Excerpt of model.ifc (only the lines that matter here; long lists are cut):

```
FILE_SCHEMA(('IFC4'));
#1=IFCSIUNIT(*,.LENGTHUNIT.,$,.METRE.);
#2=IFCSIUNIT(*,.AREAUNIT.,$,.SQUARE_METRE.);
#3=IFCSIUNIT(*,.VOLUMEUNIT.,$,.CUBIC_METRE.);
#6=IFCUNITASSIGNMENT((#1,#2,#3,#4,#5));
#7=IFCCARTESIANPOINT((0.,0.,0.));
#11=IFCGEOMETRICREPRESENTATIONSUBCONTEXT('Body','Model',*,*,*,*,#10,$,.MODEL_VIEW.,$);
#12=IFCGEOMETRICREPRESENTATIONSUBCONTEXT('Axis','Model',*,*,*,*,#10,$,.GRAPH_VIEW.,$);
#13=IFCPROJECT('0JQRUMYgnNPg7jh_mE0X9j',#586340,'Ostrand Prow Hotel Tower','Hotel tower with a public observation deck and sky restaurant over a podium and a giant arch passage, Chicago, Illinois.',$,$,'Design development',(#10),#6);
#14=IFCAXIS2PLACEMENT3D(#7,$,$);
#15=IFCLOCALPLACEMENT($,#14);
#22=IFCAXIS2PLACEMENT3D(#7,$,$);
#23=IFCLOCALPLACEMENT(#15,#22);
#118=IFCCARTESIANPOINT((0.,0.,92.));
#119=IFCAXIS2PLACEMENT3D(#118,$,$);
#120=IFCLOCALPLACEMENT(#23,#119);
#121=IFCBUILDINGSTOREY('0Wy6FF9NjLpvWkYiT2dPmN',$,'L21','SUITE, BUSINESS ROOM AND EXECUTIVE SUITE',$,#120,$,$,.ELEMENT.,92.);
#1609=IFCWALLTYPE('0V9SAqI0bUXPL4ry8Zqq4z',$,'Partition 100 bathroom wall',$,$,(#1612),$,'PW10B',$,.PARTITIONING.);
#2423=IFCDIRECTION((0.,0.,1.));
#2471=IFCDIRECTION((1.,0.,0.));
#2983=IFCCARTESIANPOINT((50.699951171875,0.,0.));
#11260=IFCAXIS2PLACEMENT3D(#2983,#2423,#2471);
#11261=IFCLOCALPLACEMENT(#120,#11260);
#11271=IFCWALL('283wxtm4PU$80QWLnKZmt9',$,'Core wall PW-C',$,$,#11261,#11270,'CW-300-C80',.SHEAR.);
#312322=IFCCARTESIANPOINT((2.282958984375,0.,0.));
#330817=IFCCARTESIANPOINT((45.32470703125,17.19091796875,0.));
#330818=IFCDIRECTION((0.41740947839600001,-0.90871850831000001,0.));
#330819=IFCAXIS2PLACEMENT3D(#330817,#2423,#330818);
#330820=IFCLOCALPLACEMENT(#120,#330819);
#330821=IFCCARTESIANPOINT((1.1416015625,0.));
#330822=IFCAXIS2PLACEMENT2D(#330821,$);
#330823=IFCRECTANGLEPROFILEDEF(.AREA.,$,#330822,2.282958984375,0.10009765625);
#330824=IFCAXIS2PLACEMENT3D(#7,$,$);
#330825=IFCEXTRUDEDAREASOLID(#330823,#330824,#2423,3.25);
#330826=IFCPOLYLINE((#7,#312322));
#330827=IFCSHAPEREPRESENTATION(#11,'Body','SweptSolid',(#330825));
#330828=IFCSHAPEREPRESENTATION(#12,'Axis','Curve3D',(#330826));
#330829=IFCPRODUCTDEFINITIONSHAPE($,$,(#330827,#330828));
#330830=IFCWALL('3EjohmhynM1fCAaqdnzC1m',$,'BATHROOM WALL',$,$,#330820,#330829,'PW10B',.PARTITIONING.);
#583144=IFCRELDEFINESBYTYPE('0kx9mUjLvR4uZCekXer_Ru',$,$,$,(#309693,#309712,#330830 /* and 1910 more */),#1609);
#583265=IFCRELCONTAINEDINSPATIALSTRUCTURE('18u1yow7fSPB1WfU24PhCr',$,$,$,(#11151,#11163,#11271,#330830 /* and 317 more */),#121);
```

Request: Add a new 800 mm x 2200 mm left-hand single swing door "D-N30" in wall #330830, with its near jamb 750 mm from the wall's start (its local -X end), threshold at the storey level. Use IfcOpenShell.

```python
import numpy as np
import ifcopenshell
import ifcopenshell.api.feature
import ifcopenshell.api.geometry
import ifcopenshell.api.root
import ifcopenshell.api.spatial
import ifcopenshell.geom
import ifcopenshell.util.element
import ifcopenshell.util.placement
import ifcopenshell.util.representation
import ifcopenshell.util.shape
import ifcopenshell.util.unit

model = ifcopenshell.open("model.ifc")
unit_scale = ifcopenshell.util.unit.calculate_unit_scale(model)
settings = ifcopenshell.geom.settings()


def volume(element):
    """Net volume in cubic metres, openings subtracted."""
    shape = ifcopenshell.geom.create_shape(settings, element)
    return ifcopenshell.util.shape.get_volume(shape.geometry)


wall = model.by_guid("3EjohmhynM1fCAaqdnzC1m")
storey = ifcopenshell.util.element.get_container(wall, ifc_class="IfcBuildingStorey")
context = ifcopenshell.util.representation.get_context(model, "Model", "Body", "MODEL_VIEW")
before = volume(wall)

width, height, from_end, sill = 0.8, 2.2, 0.75, 0.0  # metres

# The wall runs along its own X axis, and the end named is its -X end.
wall_shape = ifcopenshell.geom.create_shape(settings, wall)
x, y, z = ifcopenshell.util.shape.get_vertices(wall_shape.geometry).T
start = x.min() + from_end
face, thickness = float(y.min()), float(y.max() - y.min())
wall_matrix = ifcopenshell.util.placement.get_local_placement(wall.ObjectPlacement)
level = ifcopenshell.util.placement.get_local_placement(storey.ObjectPlacement)[2, 3]


def in_wall(x, y):
    """Placement at x, y metres in the wall's axes, at sill height."""
    matrix = wall_matrix.copy()
    matrix[:, 3] = wall_matrix @ np.array([x / unit_scale, y / unit_scale, 0.0, 1.0])
    matrix[2, 3] = level + sill / unit_scale
    return matrix


# Opening: a box that overshoots both wall faces by 50 mm.
opening = ifcopenshell.api.root.create_entity(model, ifc_class="IfcOpeningElement", predefined_type="OPENING")
box = ifcopenshell.api.geometry.add_wall_representation(
    model, context=context, length=width, height=height, thickness=thickness + 0.1
)
ifcopenshell.api.geometry.assign_representation(model, product=opening, representation=box)
ifcopenshell.api.geometry.edit_object_placement(model, product=opening, matrix=in_wall(start, face - 0.05), is_si=False)
ifcopenshell.api.feature.add_feature(model, feature=opening, element=wall)

door = ifcopenshell.api.root.create_entity(model, ifc_class="IfcDoor", name="D-N30", predefined_type="DOOR")
door.OverallWidth, door.OverallHeight = width / unit_scale, height / unit_scale
door.OperationType = "SINGLE_SWING_LEFT"
body = ifcopenshell.api.geometry.add_door_representation(
    model,
    context=context,
    overall_width=door.OverallWidth,
    overall_height=door.OverallHeight,
    operation_type="SINGLE_SWING_LEFT",
    lining_properties={"LiningDepth": thickness / unit_scale, "ThresholdDepth": thickness / unit_scale},
)
ifcopenshell.api.geometry.assign_representation(model, product=door, representation=body)
ifcopenshell.api.spatial.assign_container(model, products=[door], relating_structure=storey)
ifcopenshell.api.feature.add_filling(model, opening=opening, element=door)

# The lining spans the wall, so the door starts at the wall face.
ifcopenshell.api.geometry.edit_object_placement(model, product=door, matrix=in_wall(start, face), is_si=False)

after = volume(wall)

print(f"wall volume {before:.3f} -> {after:.3f} m3")

model.write("model_edited.ifc")
```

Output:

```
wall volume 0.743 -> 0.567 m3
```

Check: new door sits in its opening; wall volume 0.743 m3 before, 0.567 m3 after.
